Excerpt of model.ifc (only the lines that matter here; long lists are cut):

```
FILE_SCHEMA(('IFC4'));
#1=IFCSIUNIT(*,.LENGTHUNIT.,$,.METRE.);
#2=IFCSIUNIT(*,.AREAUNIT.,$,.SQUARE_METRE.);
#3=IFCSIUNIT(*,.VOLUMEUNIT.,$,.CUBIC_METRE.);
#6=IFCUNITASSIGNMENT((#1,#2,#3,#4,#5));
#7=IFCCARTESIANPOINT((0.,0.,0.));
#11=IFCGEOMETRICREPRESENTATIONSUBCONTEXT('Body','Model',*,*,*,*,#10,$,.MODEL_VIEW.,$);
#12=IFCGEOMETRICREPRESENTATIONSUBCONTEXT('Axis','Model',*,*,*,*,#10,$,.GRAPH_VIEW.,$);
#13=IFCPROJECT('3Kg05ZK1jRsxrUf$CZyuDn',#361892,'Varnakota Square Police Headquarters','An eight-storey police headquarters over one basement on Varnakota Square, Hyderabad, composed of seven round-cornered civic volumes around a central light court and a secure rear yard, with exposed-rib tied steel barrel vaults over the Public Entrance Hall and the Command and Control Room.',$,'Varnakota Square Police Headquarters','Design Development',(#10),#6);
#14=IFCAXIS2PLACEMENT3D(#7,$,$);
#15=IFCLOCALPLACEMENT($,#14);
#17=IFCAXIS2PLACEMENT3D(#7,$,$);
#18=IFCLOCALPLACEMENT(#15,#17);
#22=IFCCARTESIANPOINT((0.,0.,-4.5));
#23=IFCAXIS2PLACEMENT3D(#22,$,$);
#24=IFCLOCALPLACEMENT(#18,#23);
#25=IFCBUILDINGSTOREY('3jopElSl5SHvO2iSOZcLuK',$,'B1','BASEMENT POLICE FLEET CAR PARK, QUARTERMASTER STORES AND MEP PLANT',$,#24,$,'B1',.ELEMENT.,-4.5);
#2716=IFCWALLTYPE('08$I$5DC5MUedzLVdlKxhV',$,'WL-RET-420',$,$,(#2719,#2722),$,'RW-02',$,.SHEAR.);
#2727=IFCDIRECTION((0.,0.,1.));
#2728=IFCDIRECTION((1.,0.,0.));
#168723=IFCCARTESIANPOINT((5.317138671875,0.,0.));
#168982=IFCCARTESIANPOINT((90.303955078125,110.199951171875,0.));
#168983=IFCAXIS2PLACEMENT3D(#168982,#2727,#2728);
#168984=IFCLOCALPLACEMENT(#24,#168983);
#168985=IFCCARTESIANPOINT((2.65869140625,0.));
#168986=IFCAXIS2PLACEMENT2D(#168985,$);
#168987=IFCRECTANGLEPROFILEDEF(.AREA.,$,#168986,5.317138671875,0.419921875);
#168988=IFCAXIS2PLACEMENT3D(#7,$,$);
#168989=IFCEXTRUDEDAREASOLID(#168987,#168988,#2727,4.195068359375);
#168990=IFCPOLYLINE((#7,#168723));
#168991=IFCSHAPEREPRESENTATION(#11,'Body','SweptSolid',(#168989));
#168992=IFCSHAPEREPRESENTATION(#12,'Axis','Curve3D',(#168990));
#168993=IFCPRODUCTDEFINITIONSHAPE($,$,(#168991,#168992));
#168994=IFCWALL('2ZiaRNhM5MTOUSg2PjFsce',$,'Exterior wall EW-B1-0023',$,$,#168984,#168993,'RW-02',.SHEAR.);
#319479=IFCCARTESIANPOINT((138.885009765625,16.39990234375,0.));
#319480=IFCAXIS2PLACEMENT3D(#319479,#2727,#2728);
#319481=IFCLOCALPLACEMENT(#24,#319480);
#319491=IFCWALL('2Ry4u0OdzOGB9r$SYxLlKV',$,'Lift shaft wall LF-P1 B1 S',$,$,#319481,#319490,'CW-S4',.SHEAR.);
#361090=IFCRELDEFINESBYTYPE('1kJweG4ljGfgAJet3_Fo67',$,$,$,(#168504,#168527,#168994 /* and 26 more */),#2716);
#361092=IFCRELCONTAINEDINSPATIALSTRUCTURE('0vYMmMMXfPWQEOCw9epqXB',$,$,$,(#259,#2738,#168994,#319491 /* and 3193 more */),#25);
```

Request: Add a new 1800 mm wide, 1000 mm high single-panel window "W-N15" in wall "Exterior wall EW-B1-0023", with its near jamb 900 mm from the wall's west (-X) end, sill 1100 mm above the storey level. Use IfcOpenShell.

```python
import numpy as np
import ifcopenshell
import ifcopenshell.api.feature
import ifcopenshell.api.geometry
import ifcopenshell.api.root
import ifcopenshell.api.spatial
import ifcopenshell.geom
import ifcopenshell.util.element
import ifcopenshell.util.placement
import ifcopenshell.util.representation
import ifcopenshell.util.shape
import ifcopenshell.util.unit

model = ifcopenshell.open("model.ifc")
unit_scale = ifcopenshell.util.unit.calculate_unit_scale(model)
settings = ifcopenshell.geom.settings()


def volume(element):
    """Net volume in cubic metres, openings subtracted."""
    shape = ifcopenshell.geom.create_shape(settings, element)
    return ifcopenshell.util.shape.get_volume(shape.geometry)


wall = model.by_id(168994)
storey = ifcopenshell.util.element.get_container(wall, ifc_class="IfcBuildingStorey")
context = ifcopenshell.util.representation.get_context(model, "Model", "Body", "MODEL_VIEW")
before = volume(wall)

width, height, from_end, sill = 1.8, 1, 0.9, 1.1  # metres

# The wall runs along its own X axis, and the end named is its -X end.
wall_shape = ifcopenshell.geom.create_shape(settings, wall)
x, y, z = ifcopenshell.util.shape.get_vertices(wall_shape.geometry).T
start = x.min() + from_end
face, thickness = float(y.min()), float(y.max() - y.min())
wall_matrix = ifcopenshell.util.placement.get_local_placement(wall.ObjectPlacement)
level = ifcopenshell.util.placement.get_local_placement(storey.ObjectPlacement)[2, 3]


def in_wall(x, y):
    """Placement at x, y metres in the wall's axes, at sill height."""
    matrix = wall_matrix.copy()
    matrix[:, 3] = wall_matrix @ np.array([x / unit_scale, y / unit_scale, 0.0, 1.0])
    matrix[2, 3] = level + sill / unit_scale
    return matrix


# Opening: a box that overshoots both wall faces by 50 mm.
opening = ifcopenshell.api.root.create_entity(model, ifc_class="IfcOpeningElement", predefined_type="OPENING")
box = ifcopenshell.api.geometry.add_wall_representation(
    model, context=context, length=width, height=height, thickness=thickness + 0.1
)
ifcopenshell.api.geometry.assign_representation(model, product=opening, representation=box)
ifcopenshell.api.geometry.edit_object_placement(model, product=opening, matrix=in_wall(start, face - 0.05), is_si=False)
ifcopenshell.api.feature.add_feature(model, feature=opening, element=wall)

window = ifcopenshell.api.root.create_entity(model, ifc_class="IfcWindow", name="W-N15", predefined_type="WINDOW")
window.OverallWidth, window.OverallHeight = width / unit_scale, height / unit_scale
window.PartitioningType = "SINGLE_PANEL"
body = ifcopenshell.api.geometry.add_window_representation(
    model,
    context=context,
    overall_width=window.OverallWidth,
    overall_height=window.OverallHeight,
    partition_type="SINGLE_PANEL",
)
ifcopenshell.api.geometry.assign_representation(model, product=window, representation=body)
ifcopenshell.api.spatial.assign_container(model, products=[window], relating_structure=storey)
ifcopenshell.api.feature.add_filling(model, opening=opening, element=window)

# Centre the window in the wall's thickness.
ifcopenshell.api.geometry.edit_object_placement(model, product=window, matrix=in_wall(start, face), is_si=False)
window_shape = ifcopenshell.geom.create_shape(settings, window)
depth = ifcopenshell.util.shape.get_vertices(window_shape.geometry)[:, 1]
offset = face + thickness / 2 - (depth.min() + depth.max()) / 2
ifcopenshell.api.geometry.edit_object_placement(model, product=window, matrix=in_wall(start, offset), is_si=False)

after = volume(wall)

print(f"wall volume {before:.3f} -> {after:.3f} m3")

model.write("model_v2.ifc")
```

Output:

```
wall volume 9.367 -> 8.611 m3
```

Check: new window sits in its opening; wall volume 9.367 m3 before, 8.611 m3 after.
